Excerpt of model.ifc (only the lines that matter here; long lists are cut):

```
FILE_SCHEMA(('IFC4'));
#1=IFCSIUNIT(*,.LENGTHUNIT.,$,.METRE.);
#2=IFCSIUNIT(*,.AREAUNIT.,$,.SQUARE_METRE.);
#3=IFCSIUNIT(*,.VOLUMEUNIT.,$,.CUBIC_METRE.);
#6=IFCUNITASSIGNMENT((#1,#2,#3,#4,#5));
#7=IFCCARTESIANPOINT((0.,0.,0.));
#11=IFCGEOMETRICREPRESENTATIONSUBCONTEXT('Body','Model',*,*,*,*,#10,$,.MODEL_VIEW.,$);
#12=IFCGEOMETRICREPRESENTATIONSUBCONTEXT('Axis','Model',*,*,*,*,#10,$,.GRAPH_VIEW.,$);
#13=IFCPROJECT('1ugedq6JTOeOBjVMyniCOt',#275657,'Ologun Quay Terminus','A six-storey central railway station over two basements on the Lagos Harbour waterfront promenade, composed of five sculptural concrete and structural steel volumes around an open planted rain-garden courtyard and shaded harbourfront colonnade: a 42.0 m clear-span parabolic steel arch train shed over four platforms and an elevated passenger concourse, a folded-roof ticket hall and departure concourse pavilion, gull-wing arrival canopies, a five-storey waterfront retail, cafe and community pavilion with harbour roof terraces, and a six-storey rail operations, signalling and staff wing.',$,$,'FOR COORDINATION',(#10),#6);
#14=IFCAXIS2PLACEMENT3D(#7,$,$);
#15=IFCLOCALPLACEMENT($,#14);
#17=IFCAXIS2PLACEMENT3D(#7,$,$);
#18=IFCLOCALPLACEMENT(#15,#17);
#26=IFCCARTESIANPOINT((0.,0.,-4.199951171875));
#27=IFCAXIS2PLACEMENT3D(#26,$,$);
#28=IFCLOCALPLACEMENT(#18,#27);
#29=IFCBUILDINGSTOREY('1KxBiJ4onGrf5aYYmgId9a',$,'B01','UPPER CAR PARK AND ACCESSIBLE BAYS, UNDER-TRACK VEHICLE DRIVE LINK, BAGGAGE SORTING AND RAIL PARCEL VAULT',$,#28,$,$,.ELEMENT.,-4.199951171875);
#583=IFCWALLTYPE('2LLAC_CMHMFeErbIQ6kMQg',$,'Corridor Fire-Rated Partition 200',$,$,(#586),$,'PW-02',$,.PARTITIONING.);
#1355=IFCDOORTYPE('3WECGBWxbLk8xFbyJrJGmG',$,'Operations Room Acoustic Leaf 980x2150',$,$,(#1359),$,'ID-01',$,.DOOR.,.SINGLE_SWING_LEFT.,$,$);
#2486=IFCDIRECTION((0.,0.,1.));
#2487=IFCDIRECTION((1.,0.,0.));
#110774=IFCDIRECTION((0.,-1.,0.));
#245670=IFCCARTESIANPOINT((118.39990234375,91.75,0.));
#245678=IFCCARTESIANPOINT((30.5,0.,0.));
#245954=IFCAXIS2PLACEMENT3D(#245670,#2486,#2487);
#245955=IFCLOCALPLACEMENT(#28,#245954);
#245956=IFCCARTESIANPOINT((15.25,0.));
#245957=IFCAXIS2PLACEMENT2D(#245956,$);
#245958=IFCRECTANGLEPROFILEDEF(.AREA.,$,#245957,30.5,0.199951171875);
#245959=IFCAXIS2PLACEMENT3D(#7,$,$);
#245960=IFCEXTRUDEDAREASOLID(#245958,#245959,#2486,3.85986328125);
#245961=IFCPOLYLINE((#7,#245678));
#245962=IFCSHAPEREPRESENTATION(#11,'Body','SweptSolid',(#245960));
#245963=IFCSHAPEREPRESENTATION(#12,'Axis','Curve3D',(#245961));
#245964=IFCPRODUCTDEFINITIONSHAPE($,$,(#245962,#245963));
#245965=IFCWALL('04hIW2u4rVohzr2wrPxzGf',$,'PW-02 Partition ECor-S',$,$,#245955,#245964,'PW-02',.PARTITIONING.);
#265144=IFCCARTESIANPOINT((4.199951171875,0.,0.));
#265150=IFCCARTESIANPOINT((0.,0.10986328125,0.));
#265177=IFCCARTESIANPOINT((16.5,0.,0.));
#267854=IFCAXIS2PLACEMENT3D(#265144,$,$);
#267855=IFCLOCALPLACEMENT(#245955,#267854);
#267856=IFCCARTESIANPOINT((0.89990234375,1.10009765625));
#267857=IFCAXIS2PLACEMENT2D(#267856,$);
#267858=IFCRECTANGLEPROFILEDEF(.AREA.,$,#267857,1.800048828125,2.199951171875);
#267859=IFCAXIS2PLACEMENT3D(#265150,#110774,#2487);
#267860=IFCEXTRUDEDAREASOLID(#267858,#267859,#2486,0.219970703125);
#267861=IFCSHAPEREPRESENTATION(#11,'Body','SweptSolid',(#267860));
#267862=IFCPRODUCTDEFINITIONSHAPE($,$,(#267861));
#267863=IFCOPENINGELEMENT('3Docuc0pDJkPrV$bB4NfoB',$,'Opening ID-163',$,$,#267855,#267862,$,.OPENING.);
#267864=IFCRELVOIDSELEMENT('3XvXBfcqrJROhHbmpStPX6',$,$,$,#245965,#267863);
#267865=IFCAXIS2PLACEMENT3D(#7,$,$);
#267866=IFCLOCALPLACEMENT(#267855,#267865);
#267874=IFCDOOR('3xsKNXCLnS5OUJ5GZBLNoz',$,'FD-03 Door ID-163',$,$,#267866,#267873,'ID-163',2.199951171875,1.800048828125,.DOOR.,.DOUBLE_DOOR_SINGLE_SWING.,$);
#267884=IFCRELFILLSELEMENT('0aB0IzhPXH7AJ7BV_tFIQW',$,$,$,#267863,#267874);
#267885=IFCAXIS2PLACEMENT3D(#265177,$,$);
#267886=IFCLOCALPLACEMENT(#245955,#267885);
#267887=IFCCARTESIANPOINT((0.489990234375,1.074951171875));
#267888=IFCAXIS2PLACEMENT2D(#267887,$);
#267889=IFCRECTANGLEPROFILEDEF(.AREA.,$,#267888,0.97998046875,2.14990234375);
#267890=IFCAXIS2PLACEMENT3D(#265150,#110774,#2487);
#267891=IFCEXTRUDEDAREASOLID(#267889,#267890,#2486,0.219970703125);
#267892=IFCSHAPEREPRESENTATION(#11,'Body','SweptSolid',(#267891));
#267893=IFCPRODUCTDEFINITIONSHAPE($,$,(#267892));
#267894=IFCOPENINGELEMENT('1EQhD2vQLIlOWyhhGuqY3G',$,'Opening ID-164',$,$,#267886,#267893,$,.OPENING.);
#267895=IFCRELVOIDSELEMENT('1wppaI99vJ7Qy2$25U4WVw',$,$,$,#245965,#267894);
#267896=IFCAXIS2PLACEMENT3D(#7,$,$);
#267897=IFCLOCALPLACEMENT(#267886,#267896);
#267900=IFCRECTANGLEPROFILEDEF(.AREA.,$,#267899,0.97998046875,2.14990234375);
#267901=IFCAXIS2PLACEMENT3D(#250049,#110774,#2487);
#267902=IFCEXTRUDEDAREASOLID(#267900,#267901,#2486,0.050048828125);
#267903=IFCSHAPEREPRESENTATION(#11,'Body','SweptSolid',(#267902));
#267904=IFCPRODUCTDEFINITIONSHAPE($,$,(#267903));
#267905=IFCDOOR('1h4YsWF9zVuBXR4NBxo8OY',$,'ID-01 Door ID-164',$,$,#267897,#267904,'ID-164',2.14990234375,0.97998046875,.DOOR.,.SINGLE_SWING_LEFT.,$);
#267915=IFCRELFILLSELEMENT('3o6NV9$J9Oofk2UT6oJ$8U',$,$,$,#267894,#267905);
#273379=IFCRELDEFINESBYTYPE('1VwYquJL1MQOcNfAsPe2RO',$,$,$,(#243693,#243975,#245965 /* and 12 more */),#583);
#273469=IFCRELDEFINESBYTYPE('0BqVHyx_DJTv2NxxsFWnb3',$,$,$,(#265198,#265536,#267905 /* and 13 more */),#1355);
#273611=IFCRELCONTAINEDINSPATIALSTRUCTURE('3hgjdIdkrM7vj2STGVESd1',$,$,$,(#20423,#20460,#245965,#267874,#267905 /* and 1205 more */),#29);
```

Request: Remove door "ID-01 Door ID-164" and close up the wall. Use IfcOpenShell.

```python
import ifcopenshell
import ifcopenshell.api.feature
import ifcopenshell.api.root
import ifcopenshell.geom
import ifcopenshell.util.shape

model = ifcopenshell.open("model.ifc")
settings = ifcopenshell.geom.settings()


def volume(element):
    """Net volume in cubic metres, openings subtracted."""
    shape = ifcopenshell.geom.create_shape(settings, element)
    return ifcopenshell.util.shape.get_volume(shape.geometry)


door = model.by_guid("1h4YsWF9zVuBXR4NBxo8OY")
opening = door.FillsVoids[0].RelatingOpeningElement
wall = opening.VoidsElements[0].RelatingBuildingElement
before = volume(wall)

ifcopenshell.api.root.remove_product(model, product=door)
ifcopenshell.api.feature.remove_feature(model, feature=opening)

after = volume(wall)

print(f"wall volume {before:.3f} -> {after:.3f} m3")

model.write("model-out.ifc")
```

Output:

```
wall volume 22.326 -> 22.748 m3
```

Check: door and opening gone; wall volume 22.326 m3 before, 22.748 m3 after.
